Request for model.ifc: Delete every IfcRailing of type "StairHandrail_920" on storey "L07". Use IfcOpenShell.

First a look at what the model holds.

```python
import ifcopenshell
import ifcopenshell.util.element

model = ifcopenshell.open("model.ifc")
print(model.schema)
storey = next(s for s in model.by_type("IfcBuildingStorey") if s.Name == "L07")
railings = [e for e in ifcopenshell.util.element.get_decomposition(storey) if e.is_a("IfcRailing")]
seen = {}
for e in railings:
    element_type = ifcopenshell.util.element.get_type(e)
    name = element_type.Name if element_type not in (None, e) else None
    seen[name] = seen.get(name, 0) + 1
for name, count in sorted(seen.items(), key=str):
    print(count, "x", name)
```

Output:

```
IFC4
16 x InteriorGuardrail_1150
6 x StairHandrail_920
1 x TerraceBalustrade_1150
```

```python
import ifcopenshell
import ifcopenshell.api.root
import ifcopenshell.util.element

model = ifcopenshell.open("model.ifc")

storey = next(s for s in model.by_type("IfcBuildingStorey") if s.Name == "L07")
railings = [e for e in ifcopenshell.util.element.get_decomposition(storey) if e.is_a("IfcRailing")]
targets = [e for e in railings if (t := ifcopenshell.util.element.get_type(e)) not in (None, e) and t.Name == "StairHandrail_920"]

for e in targets:
    ifcopenshell.api.root.remove_product(model, product=e)
print(len(targets), "removed")

model.write("model_edited.ifc")
```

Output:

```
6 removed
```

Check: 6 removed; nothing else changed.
